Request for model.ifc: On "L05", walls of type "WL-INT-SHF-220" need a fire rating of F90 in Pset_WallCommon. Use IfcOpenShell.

First a look at what the model holds.

```python
import ifcopenshell
import ifcopenshell.util.element

model = ifcopenshell.open("model.ifc")
print(model.schema)
storey = next(s for s in model.by_type("IfcBuildingStorey") if s.Name == "L05")
walls = [e for e in ifcopenshell.util.element.get_decomposition(storey) if e.is_a("IfcWall")]
seen = {}
for e in walls:
    element_type = ifcopenshell.util.element.get_type(e)
    key = (element_type.Name if element_type != e and element_type else None, ifcopenshell.util.element.get_pset(e, "Pset_WallCommon", "FireRating"))
    seen[key] = seen.get(key, 0) + 1
for (name, value), count in sorted(seen.items(), key=str):
    print(count, "x", name, "|", value)
```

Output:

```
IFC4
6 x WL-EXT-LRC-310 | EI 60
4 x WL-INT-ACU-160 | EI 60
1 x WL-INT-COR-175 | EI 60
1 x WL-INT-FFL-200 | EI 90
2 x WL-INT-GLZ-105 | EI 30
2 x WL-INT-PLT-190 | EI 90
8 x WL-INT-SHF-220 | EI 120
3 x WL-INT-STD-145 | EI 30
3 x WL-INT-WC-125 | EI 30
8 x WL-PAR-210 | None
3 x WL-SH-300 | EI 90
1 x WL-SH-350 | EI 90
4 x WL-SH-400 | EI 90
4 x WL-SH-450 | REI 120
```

```python
import ifcopenshell
import ifcopenshell.api.pset
import ifcopenshell.util.element

model = ifcopenshell.open("model.ifc")

storey = next(s for s in model.by_type("IfcBuildingStorey") if s.Name == "L05")
walls = [e for e in ifcopenshell.util.element.get_decomposition(storey) if e.is_a("IfcWall")]

count = 0
for e in walls:
    element_type = ifcopenshell.util.element.get_type(e)
    if element_type in (None, e) or element_type.Name != "WL-INT-SHF-220":
        continue
    # add_pset returns the element's existing set when there is one.
    pset = ifcopenshell.api.pset.add_pset(model, product=e, name="Pset_WallCommon")
    ifcopenshell.api.pset.edit_pset(model, pset=pset, properties={"FireRating": "F90"})
    count += 1

print(count, "walls updated")

model.write("model_edited.ifc")
```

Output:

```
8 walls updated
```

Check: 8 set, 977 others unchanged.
